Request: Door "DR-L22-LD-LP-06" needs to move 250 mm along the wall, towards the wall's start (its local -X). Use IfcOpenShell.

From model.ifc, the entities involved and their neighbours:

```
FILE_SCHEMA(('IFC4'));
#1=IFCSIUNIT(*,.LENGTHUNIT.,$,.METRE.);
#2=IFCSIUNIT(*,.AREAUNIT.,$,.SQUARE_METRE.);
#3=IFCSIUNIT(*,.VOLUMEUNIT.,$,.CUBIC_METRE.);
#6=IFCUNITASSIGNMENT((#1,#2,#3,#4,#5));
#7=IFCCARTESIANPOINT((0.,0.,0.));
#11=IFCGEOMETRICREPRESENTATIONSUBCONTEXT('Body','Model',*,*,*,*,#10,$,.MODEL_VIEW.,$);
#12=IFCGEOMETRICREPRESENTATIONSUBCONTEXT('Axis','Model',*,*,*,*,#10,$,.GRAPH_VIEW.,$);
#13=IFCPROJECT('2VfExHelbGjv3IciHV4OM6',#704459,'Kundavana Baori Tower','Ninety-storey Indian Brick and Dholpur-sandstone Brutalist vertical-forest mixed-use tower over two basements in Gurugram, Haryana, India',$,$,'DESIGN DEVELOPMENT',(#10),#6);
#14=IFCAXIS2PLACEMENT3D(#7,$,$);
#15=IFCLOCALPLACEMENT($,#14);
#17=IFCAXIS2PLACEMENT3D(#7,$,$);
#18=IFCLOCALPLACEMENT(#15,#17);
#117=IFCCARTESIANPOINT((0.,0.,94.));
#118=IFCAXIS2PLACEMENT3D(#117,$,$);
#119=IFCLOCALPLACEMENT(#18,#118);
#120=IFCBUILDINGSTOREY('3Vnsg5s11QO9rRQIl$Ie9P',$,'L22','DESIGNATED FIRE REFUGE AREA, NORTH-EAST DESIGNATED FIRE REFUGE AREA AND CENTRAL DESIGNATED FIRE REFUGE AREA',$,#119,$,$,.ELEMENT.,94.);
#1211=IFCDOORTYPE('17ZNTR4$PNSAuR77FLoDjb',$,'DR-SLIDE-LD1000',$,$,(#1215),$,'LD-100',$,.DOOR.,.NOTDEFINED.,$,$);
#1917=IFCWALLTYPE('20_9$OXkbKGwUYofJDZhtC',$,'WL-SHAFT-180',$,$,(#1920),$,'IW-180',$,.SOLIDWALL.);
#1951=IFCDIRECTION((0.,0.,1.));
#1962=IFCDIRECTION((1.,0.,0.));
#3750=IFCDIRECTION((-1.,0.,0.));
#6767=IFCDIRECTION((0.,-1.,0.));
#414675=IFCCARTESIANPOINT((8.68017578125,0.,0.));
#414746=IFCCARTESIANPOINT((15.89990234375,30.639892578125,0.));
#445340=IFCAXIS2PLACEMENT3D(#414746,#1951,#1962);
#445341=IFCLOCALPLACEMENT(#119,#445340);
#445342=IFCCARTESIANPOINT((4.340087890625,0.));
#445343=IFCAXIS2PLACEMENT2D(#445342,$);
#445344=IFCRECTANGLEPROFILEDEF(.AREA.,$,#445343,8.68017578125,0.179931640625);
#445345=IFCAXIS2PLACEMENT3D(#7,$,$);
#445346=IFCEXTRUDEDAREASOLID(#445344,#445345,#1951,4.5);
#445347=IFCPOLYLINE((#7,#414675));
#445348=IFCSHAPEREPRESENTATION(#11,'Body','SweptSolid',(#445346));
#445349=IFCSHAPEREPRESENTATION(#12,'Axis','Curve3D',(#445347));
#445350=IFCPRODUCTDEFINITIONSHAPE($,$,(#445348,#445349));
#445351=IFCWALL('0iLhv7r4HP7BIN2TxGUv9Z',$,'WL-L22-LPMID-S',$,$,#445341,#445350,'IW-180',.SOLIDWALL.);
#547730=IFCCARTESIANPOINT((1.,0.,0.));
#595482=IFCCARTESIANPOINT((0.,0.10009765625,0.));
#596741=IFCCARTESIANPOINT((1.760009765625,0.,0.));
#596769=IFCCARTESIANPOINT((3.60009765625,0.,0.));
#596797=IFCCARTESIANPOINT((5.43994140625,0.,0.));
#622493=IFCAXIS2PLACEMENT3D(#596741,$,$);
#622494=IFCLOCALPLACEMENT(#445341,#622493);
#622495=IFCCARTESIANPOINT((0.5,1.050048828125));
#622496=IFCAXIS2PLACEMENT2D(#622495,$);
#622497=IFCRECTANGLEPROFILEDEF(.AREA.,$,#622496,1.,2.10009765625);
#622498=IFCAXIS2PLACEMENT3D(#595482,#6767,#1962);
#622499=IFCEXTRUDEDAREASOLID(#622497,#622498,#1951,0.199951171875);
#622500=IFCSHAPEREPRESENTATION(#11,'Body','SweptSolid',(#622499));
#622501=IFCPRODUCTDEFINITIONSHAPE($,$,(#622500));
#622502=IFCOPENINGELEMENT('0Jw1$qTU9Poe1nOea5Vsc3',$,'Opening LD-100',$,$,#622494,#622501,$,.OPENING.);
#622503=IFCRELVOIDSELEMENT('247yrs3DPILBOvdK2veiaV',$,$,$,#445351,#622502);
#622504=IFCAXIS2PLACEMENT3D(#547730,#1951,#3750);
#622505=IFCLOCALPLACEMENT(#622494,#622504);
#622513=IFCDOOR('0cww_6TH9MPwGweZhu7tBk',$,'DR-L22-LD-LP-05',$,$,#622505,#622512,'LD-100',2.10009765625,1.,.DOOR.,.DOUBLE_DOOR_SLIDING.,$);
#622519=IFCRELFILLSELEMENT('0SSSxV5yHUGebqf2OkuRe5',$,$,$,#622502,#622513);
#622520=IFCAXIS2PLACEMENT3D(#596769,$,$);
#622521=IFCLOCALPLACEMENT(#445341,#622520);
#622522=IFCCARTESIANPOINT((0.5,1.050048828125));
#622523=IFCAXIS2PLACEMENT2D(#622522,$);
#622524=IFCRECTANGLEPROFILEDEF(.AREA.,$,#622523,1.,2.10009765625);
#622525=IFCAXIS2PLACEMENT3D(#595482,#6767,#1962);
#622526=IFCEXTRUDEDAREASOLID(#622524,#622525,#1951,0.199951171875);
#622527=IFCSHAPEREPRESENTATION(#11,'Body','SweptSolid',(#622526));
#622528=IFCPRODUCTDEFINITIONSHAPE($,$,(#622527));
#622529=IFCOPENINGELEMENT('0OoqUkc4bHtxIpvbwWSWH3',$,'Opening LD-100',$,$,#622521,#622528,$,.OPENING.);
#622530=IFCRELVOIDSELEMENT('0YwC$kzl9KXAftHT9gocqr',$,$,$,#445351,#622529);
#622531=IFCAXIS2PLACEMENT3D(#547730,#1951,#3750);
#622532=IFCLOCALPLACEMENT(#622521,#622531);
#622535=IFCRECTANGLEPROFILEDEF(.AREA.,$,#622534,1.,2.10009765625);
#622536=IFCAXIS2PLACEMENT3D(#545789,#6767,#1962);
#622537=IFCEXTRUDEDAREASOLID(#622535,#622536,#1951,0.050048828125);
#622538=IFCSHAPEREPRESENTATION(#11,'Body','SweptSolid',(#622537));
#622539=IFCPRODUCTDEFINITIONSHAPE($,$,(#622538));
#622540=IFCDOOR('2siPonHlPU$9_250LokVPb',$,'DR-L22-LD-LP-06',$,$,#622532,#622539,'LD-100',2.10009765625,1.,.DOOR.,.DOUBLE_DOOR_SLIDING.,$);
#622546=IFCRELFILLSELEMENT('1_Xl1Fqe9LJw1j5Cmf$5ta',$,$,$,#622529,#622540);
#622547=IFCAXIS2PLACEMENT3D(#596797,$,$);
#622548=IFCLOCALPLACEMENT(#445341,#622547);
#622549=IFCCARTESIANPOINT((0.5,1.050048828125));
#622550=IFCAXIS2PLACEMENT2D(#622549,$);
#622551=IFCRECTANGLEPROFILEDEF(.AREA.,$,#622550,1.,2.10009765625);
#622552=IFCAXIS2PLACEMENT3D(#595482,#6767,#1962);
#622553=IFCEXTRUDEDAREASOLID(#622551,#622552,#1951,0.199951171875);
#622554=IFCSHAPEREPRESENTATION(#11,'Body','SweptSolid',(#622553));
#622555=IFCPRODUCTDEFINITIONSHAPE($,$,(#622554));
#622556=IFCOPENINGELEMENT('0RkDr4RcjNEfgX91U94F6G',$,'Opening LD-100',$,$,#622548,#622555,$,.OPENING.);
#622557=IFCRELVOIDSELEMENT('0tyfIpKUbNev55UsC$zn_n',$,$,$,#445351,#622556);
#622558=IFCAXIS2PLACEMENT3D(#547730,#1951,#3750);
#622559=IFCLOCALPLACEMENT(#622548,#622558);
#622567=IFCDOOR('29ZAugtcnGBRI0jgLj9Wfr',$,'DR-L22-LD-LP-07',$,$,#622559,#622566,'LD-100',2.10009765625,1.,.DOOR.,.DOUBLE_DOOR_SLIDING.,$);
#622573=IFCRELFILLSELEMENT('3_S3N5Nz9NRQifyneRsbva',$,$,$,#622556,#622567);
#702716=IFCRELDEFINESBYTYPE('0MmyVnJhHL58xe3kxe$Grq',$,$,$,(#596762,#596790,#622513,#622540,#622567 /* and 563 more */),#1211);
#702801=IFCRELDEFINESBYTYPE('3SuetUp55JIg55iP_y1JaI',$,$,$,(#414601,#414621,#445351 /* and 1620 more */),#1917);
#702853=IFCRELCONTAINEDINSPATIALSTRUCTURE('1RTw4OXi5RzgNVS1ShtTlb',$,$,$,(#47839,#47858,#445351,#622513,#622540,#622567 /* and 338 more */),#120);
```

```python
import ifcopenshell
import ifcopenshell.api.geometry
import ifcopenshell.util.placement
import ifcopenshell.util.unit

model = ifcopenshell.open("model.ifc")
unit_scale = ifcopenshell.util.unit.calculate_unit_scale(model)

door = model.by_guid("2siPonHlPU$9_250LokVPb")
opening = door.FillsVoids[0].RelatingOpeningElement
wall = opening.VoidsElements[0].RelatingBuildingElement

wall_matrix = ifcopenshell.util.placement.get_local_placement(wall.ObjectPlacement)
shift = wall_matrix[:3, 0] * -0.25 / unit_scale
before = ifcopenshell.util.placement.get_local_placement(door.ObjectPlacement)[:3, 3].copy()

# The door is placed relative to its opening, so it follows when the opening moves.
matrix = ifcopenshell.util.placement.get_local_placement(opening.ObjectPlacement)
matrix[:3, 3] += shift
ifcopenshell.api.geometry.edit_object_placement(
    model, product=opening, matrix=matrix, is_si=False, should_transform_children=True
)

after = ifcopenshell.util.placement.get_local_placement(door.ObjectPlacement)[:3, 3]
print("door moved by", (after - before).round(3) + 0.0)

model.write("model-out.ifc")
```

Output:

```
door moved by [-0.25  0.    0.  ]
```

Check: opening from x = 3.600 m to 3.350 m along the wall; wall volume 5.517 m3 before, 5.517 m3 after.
